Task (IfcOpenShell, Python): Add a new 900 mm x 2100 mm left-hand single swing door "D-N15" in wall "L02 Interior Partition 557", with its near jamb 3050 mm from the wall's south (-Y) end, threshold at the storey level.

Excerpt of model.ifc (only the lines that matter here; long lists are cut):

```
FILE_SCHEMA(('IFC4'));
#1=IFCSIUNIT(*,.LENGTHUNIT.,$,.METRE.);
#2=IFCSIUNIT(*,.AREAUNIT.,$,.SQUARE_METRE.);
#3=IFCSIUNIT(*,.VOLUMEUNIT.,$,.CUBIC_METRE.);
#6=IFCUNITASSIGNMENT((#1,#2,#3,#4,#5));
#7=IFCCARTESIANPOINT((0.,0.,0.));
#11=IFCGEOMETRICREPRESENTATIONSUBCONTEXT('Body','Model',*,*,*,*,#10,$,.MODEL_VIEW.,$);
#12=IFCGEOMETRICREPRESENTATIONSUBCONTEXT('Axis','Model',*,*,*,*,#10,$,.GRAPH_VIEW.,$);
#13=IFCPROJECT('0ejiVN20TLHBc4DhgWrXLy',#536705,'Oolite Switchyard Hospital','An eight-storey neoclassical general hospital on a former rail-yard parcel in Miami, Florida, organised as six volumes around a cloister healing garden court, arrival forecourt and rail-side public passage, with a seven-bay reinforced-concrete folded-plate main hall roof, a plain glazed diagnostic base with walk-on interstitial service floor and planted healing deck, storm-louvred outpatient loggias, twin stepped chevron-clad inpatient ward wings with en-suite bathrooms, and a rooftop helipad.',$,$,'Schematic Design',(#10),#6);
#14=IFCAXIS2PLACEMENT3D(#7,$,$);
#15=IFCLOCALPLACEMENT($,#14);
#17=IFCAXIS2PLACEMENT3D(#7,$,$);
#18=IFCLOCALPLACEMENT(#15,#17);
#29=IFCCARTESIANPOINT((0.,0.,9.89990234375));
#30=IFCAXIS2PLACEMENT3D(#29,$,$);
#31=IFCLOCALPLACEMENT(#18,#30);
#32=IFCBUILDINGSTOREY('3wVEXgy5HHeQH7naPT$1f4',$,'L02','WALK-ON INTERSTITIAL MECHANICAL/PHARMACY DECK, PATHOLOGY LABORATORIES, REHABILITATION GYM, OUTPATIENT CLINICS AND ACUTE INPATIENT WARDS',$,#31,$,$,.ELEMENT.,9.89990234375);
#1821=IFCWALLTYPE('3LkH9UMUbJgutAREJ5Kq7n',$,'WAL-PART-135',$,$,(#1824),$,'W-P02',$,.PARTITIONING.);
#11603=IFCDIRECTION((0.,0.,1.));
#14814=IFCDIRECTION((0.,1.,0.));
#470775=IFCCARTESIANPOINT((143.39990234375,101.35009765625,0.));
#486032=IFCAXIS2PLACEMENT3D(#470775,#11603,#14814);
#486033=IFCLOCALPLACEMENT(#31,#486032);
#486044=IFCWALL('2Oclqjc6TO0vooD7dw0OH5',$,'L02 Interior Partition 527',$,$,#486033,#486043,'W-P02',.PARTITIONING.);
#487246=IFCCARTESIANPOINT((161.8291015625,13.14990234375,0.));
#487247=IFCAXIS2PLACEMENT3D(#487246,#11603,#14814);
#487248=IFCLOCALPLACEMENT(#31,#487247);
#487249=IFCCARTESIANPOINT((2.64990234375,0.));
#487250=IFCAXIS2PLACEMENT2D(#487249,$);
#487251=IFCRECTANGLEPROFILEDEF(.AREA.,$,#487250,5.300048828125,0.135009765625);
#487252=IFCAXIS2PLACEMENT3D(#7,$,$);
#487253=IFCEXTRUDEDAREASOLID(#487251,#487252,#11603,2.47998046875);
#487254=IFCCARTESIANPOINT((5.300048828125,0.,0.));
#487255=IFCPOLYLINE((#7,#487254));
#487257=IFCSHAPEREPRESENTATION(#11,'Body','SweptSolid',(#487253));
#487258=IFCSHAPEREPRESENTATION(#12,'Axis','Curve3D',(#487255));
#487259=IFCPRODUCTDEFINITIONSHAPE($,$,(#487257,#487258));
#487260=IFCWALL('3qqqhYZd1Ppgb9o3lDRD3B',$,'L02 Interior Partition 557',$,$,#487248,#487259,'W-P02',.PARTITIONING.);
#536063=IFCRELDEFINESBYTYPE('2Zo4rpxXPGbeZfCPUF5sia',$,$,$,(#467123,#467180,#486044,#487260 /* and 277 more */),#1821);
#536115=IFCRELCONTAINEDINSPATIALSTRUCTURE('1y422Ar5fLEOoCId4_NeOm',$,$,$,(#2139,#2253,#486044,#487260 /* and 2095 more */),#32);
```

```python
import numpy as np
import ifcopenshell
import ifcopenshell.api.feature
import ifcopenshell.api.geometry
import ifcopenshell.api.root
import ifcopenshell.api.spatial
import ifcopenshell.geom
import ifcopenshell.util.element
import ifcopenshell.util.placement
import ifcopenshell.util.representation
import ifcopenshell.util.shape
import ifcopenshell.util.unit

model = ifcopenshell.open("model.ifc")
unit_scale = ifcopenshell.util.unit.calculate_unit_scale(model)
settings = ifcopenshell.geom.settings()


def volume(element):
    """Net volume in cubic metres, openings subtracted."""
    shape = ifcopenshell.geom.create_shape(settings, element)
    return ifcopenshell.util.shape.get_volume(shape.geometry)


wall = model.by_guid("3qqqhYZd1Ppgb9o3lDRD3B")
storey = ifcopenshell.util.element.get_container(wall, ifc_class="IfcBuildingStorey")
context = ifcopenshell.util.representation.get_context(model, "Model", "Body", "MODEL_VIEW")
before = volume(wall)

width, height, from_end, sill = 0.9, 2.1, 3.05, 0.0  # metres

# The wall runs along its own X axis, and the end named is its -X end.
wall_shape = ifcopenshell.geom.create_shape(settings, wall)
x, y, z = ifcopenshell.util.shape.get_vertices(wall_shape.geometry).T
start = x.min() + from_end
face, thickness = float(y.min()), float(y.max() - y.min())
wall_matrix = ifcopenshell.util.placement.get_local_placement(wall.ObjectPlacement)
level = ifcopenshell.util.placement.get_local_placement(storey.ObjectPlacement)[2, 3]


def in_wall(x, y):
    """Placement at x, y metres in the wall's axes, at sill height."""
    matrix = wall_matrix.copy()
    matrix[:, 3] = wall_matrix @ np.array([x / unit_scale, y / unit_scale, 0.0, 1.0])
    matrix[2, 3] = level + sill / unit_scale
    return matrix


# Opening: a box that overshoots both wall faces by 50 mm.
opening = ifcopenshell.api.root.create_entity(model, ifc_class="IfcOpeningElement", predefined_type="OPENING")
box = ifcopenshell.api.geometry.add_wall_representation(
    model, context=context, length=width, height=height, thickness=thickness + 0.1
)
ifcopenshell.api.geometry.assign_representation(model, product=opening, representation=box)
ifcopenshell.api.geometry.edit_object_placement(model, product=opening, matrix=in_wall(start, face - 0.05), is_si=False)
ifcopenshell.api.feature.add_feature(model, feature=opening, element=wall)

door = ifcopenshell.api.root.create_entity(model, ifc_class="IfcDoor", name="D-N15", predefined_type="DOOR")
door.OverallWidth, door.OverallHeight = width / unit_scale, height / unit_scale
door.OperationType = "SINGLE_SWING_LEFT"
body = ifcopenshell.api.geometry.add_door_representation(
    model,
    context=context,
    overall_width=door.OverallWidth,
    overall_height=door.OverallHeight,
    operation_type="SINGLE_SWING_LEFT",
    lining_properties={"LiningDepth": thickness / unit_scale, "ThresholdDepth": thickness / unit_scale},
)
ifcopenshell.api.geometry.assign_representation(model, product=door, representation=body)
ifcopenshell.api.spatial.assign_container(model, products=[door], relating_structure=storey)
ifcopenshell.api.feature.add_filling(model, opening=opening, element=door)

# The lining spans the wall, so the door starts at the wall face.
ifcopenshell.api.geometry.edit_object_placement(model, product=door, matrix=in_wall(start, face), is_si=False)

after = volume(wall)

print(f"wall volume {before:.3f} -> {after:.3f} m3")

model.write("model_rev.ifc")
```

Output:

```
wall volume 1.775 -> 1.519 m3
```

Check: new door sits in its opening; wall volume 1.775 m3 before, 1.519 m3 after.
